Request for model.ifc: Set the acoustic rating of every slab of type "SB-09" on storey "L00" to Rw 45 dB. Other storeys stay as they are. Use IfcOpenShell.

First a look at what the model holds.

```python
import ifcopenshell
import ifcopenshell.util.element

model = ifcopenshell.open("model.ifc")
print(model.schema)
storey = next(s for s in model.by_type("IfcBuildingStorey") if s.Name == "L00")
slabs = [e for e in ifcopenshell.util.element.get_decomposition(storey) if e.is_a("IfcSlab")]
seen = {}
for e in slabs:
    element_type = ifcopenshell.util.element.get_type(e)
    key = (element_type.Name if element_type != e and element_type else None, ifcopenshell.util.element.get_pset(e, "Pset_SlabCommon", "AcousticRating"))
    seen[key] = seen.get(key, 0) + 1
for (name, value), count in sorted(seen.items(), key=str):
    print(count, "x", name, "|", value)
```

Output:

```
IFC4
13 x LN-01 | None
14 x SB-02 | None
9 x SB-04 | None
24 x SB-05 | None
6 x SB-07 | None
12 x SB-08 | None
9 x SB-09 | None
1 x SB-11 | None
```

```python
import ifcopenshell
import ifcopenshell.api.pset
import ifcopenshell.util.element

model = ifcopenshell.open("model.ifc")

storey = next(s for s in model.by_type("IfcBuildingStorey") if s.Name == "L00")
slabs = [e for e in ifcopenshell.util.element.get_decomposition(storey) if e.is_a("IfcSlab")]

count = 0
for e in slabs:
    element_type = ifcopenshell.util.element.get_type(e)
    if element_type in (None, e) or element_type.Name != "SB-09":
        continue
    # add_pset returns the element's existing set when there is one.
    pset = ifcopenshell.api.pset.add_pset(model, product=e, name="Pset_SlabCommon")
    ifcopenshell.api.pset.edit_pset(model, pset=pset, properties={"AcousticRating": "Rw 45 dB"})
    count += 1

print(count, "slabs updated")

model.write("model_edited.ifc")
```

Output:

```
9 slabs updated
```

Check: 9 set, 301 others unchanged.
